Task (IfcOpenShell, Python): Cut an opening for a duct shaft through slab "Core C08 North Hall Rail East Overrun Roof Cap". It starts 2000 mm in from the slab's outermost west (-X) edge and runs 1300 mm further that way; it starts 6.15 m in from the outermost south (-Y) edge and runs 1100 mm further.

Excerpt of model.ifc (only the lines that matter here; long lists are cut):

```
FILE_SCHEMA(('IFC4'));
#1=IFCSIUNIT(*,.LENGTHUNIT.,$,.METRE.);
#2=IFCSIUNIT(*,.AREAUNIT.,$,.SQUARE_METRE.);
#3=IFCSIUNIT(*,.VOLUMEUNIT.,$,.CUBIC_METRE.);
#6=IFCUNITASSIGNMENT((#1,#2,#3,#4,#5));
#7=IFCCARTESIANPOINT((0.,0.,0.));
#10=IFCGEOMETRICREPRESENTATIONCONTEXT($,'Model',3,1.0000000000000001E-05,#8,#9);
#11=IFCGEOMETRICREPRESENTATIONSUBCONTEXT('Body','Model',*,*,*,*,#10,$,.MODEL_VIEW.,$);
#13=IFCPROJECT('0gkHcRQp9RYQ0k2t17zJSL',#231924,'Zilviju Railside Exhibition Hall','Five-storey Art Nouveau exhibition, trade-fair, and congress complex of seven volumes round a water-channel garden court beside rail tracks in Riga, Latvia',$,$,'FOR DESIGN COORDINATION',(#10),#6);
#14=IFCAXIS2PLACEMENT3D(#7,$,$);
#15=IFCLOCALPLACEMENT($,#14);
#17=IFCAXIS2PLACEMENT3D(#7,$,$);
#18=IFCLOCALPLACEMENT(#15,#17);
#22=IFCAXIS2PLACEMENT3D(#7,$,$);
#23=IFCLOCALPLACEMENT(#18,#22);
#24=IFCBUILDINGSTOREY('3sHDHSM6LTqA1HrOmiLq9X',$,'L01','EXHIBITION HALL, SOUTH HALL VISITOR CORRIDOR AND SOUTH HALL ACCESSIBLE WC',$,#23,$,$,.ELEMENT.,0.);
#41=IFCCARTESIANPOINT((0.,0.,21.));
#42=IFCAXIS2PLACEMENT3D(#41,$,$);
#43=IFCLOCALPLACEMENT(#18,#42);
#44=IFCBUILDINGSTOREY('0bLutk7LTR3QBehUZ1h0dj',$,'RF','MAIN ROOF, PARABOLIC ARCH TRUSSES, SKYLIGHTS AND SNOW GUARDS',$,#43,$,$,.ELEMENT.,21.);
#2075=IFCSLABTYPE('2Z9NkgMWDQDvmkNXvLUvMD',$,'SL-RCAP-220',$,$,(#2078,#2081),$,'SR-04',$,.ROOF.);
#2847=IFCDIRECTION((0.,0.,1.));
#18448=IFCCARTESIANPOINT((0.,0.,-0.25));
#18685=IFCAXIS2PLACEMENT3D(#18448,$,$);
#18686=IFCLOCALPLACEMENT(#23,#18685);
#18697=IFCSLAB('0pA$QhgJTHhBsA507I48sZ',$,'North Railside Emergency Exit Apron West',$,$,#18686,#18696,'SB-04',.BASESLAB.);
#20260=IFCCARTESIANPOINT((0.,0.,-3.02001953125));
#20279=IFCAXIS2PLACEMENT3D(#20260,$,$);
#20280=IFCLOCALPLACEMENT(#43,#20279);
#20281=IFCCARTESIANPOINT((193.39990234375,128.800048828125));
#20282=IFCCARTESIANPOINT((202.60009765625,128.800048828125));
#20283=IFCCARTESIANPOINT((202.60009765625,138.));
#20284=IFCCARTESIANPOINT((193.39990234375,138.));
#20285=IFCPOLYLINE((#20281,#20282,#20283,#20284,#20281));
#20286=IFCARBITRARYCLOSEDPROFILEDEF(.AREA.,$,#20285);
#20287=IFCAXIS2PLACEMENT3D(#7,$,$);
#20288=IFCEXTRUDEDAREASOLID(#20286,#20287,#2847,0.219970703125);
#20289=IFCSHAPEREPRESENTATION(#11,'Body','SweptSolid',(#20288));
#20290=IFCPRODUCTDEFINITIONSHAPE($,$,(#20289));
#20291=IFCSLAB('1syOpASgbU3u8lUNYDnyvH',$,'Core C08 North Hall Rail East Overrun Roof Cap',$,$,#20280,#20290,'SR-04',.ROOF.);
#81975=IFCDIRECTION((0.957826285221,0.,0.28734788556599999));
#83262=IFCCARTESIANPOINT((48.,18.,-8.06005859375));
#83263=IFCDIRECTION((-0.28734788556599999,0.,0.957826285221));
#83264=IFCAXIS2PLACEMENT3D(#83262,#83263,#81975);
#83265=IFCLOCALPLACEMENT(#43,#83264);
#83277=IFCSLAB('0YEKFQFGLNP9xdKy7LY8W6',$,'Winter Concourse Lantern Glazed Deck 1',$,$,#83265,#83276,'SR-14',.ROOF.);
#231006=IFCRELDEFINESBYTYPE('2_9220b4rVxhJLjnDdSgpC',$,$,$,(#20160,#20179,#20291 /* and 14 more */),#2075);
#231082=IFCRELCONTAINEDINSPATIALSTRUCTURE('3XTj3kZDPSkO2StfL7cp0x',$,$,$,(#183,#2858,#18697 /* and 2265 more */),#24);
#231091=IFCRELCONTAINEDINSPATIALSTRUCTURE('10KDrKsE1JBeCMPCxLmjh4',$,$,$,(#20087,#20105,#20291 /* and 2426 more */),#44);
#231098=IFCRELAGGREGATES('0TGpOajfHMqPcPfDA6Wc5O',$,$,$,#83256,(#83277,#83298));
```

```python
import numpy as np
import ifcopenshell
import ifcopenshell.api.feature
import ifcopenshell.api.geometry
import ifcopenshell.api.root
import ifcopenshell.geom
import ifcopenshell.util.placement
import ifcopenshell.util.representation
import ifcopenshell.util.shape
import ifcopenshell.util.unit

model = ifcopenshell.open("model.ifc")
unit_scale = ifcopenshell.util.unit.calculate_unit_scale(model)
settings = ifcopenshell.geom.settings()


def volume(element):
    """Net volume in cubic metres, openings subtracted."""
    shape = ifcopenshell.geom.create_shape(settings, element)
    return ifcopenshell.util.shape.get_volume(shape.geometry)


slab = model.by_guid("1syOpASgbU3u8lUNYDnyvH")
before = volume(slab)

# Extent in the slab's own axes, in metres. The edges named are its -X and -Y sides.
slab_shape = ifcopenshell.geom.create_shape(settings, slab)
vertices = ifcopenshell.util.shape.get_vertices(slab_shape.geometry)
x_min, y_min, bottom = vertices.min(axis=0)
top = vertices[:, 2].max()

opening = ifcopenshell.api.root.create_entity(model, ifc_class="IfcOpeningElement", name="Duct shaft opening", predefined_type="OPENING")
context = ifcopenshell.util.representation.get_context(model, "Model", "Body", "MODEL_VIEW")
width, depth = 1.3, 1.1
outline = [(0.0, 0.0), (width, 0.0), (width, depth), (0.0, depth), (0.0, 0.0)]
# Overshoot both faces by 50 mm so the cut is clean.
shape = ifcopenshell.api.geometry.add_slab_representation(
    model, context=context, depth=top - bottom + 0.1, polyline=outline
)
ifcopenshell.api.geometry.assign_representation(model, product=opening, representation=shape)

matrix = ifcopenshell.util.placement.get_local_placement(slab.ObjectPlacement)
matrix[:, 3] = matrix @ np.append(np.array([x_min + 2, y_min + 6.15, bottom - 0.05]) / unit_scale, 1.0)
ifcopenshell.api.geometry.edit_object_placement(model, product=opening, matrix=matrix, is_si=False)
ifcopenshell.api.feature.add_feature(model, feature=opening, element=slab)

after = volume(slab)

print(f"slab volume {before:.3f} -> {after:.3f} m3")

model.write("model-out.ifc")
```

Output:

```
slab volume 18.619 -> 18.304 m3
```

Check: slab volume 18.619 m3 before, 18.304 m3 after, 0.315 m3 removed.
